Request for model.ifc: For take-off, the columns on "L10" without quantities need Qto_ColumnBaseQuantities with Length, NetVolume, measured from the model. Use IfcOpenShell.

First a look at what the model holds.

```python
import ifcopenshell
import ifcopenshell.util.element
import ifcopenshell.util.unit

model = ifcopenshell.open("model.ifc")
print(model.schema)
for unit_type in ("LENGTHUNIT", "AREAUNIT", "VOLUMEUNIT"):
    print(unit_type, ifcopenshell.util.unit.calculate_unit_scale(model, unit_type))
storey = next(s for s in model.by_type("IfcBuildingStorey") if s.Name == "L10")
columns = [e for e in ifcopenshell.util.element.get_decomposition(storey) if e.is_a("IfcColumn")]
for e in sorted(columns, key=lambda e: e.id()):
    print(e.id(), e.is_a(), e.Name, list(ifcopenshell.util.element.get_psets(e, qtos_only=True)), sep=" | ")
```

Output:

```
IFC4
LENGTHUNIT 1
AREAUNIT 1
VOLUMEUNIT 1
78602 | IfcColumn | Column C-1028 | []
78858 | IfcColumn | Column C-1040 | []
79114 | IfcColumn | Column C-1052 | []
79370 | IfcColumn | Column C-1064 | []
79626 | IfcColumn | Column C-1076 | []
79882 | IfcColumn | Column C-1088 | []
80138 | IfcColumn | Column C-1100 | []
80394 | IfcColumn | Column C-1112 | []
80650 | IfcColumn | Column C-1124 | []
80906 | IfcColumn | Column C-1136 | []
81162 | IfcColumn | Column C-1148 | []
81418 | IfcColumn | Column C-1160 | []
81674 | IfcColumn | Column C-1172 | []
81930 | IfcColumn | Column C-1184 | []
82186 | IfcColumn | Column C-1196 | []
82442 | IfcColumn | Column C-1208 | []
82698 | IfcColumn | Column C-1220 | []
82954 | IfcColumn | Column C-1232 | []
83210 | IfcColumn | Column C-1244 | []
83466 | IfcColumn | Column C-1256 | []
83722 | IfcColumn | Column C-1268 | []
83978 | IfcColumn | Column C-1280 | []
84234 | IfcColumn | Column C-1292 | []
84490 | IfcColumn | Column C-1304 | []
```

```python
import ifcopenshell
import ifcopenshell.api.pset
import ifcopenshell.geom
import ifcopenshell.util.element
import ifcopenshell.util.shape
import ifcopenshell.util.unit

model = ifcopenshell.open("model.ifc")
unit_scale = ifcopenshell.util.unit.calculate_unit_scale(model)
volume_scale = ifcopenshell.util.unit.calculate_unit_scale(model, "VOLUMEUNIT")
settings = ifcopenshell.geom.settings()

storey = next(s for s in model.by_type("IfcBuildingStorey") if s.Name == "L10")
columns = [e for e in ifcopenshell.util.element.get_decomposition(storey) if e.is_a("IfcColumn")]

for e in sorted(columns, key=lambda e: e.id()):
    if ifcopenshell.util.element.get_psets(e, qtos_only=True, should_inherit=False):
        continue
    # Geometry comes back in metres, in the element's own axes.
    shape = ifcopenshell.geom.create_shape(settings, e)
    values = {
        "Length": ifcopenshell.util.shape.get_z(shape.geometry) / unit_scale,
        "NetVolume": ifcopenshell.util.shape.get_volume(shape.geometry) / volume_scale,
    }
    qto = ifcopenshell.api.pset.add_qto(model, product=e, name="Qto_ColumnBaseQuantities")
    ifcopenshell.api.pset.edit_qto(model, qto=qto, properties=values)
    print(e.id(), {k: round(v, 3) for k, v in values.items()})

model.write("model_rev.ifc")
```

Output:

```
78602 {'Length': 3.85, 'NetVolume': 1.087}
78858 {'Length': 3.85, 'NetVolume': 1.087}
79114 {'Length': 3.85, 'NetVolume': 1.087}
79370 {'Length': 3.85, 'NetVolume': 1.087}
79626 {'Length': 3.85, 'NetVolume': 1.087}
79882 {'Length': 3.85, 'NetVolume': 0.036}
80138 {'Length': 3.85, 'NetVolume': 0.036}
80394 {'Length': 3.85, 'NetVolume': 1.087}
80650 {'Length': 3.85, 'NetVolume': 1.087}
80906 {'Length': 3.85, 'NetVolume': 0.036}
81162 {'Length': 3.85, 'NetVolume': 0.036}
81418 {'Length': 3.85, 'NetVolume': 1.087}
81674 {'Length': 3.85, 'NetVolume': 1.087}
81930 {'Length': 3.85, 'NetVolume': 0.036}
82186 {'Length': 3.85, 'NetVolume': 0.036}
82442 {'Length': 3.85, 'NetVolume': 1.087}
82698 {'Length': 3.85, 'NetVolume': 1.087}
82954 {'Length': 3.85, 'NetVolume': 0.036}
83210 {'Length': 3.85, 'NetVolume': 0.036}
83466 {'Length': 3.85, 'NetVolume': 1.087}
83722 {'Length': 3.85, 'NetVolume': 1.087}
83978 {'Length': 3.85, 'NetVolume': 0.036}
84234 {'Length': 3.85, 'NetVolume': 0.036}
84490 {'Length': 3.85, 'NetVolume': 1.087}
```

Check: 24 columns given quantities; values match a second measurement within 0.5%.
